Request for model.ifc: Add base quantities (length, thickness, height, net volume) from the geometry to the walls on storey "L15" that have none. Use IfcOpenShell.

First a look at what the model holds.

```python
import ifcopenshell
import ifcopenshell.util.element
import ifcopenshell.util.unit

model = ifcopenshell.open("model.ifc")
print(model.schema)
for unit_type in ("LENGTHUNIT", "AREAUNIT", "VOLUMEUNIT"):
    print(unit_type, ifcopenshell.util.unit.calculate_unit_scale(model, unit_type))
storey = next(s for s in model.by_type("IfcBuildingStorey") if s.Name == "L15")
walls = [e for e in ifcopenshell.util.element.get_decomposition(storey) if e.is_a("IfcWall")]
for e in sorted(walls, key=lambda e: e.id()):
    print(e.id(), e.is_a(), e.Name, list(ifcopenshell.util.element.get_psets(e, qtos_only=True)), sep=" | ")
```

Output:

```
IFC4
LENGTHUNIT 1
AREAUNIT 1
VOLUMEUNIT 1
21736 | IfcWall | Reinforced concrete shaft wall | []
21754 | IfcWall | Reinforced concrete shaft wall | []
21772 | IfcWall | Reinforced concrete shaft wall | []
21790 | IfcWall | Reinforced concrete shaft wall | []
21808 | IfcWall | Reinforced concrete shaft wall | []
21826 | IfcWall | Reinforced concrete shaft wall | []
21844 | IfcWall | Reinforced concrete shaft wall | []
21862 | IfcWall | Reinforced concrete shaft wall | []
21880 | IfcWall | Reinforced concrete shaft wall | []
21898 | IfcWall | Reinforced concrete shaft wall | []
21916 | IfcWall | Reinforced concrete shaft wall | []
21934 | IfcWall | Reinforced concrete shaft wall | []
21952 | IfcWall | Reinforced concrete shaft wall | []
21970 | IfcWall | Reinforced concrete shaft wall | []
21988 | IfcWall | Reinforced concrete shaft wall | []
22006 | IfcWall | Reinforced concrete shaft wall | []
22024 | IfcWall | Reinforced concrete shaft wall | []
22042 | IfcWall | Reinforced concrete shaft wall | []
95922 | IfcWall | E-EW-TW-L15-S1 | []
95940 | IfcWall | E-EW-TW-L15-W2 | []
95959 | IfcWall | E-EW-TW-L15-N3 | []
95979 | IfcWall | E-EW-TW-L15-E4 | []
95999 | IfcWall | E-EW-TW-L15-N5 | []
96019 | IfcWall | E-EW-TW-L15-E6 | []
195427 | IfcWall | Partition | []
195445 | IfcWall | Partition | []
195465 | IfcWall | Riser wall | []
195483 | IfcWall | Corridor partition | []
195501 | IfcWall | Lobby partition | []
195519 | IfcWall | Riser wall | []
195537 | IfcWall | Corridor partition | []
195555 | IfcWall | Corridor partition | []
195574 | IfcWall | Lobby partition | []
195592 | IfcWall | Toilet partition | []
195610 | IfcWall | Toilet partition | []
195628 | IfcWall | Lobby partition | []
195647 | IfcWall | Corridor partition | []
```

```python
import ifcopenshell
import ifcopenshell.api.pset
import ifcopenshell.geom
import ifcopenshell.util.element
import ifcopenshell.util.shape
import ifcopenshell.util.unit

model = ifcopenshell.open("model.ifc")
unit_scale = ifcopenshell.util.unit.calculate_unit_scale(model)
volume_scale = ifcopenshell.util.unit.calculate_unit_scale(model, "VOLUMEUNIT")
settings = ifcopenshell.geom.settings()

storey = next(s for s in model.by_type("IfcBuildingStorey") if s.Name == "L15")
walls = [e for e in ifcopenshell.util.element.get_decomposition(storey) if e.is_a("IfcWall")]

for e in sorted(walls, key=lambda e: e.id()):
    if ifcopenshell.util.element.get_psets(e, qtos_only=True, should_inherit=False):
        continue
    # Geometry comes back in metres, in the element's own axes.
    shape = ifcopenshell.geom.create_shape(settings, e)
    values = {
        "Length": ifcopenshell.util.shape.get_x(shape.geometry) / unit_scale,
        "Width": ifcopenshell.util.shape.get_y(shape.geometry) / unit_scale,
        "Height": ifcopenshell.util.shape.get_z(shape.geometry) / unit_scale,
        "NetVolume": ifcopenshell.util.shape.get_volume(shape.geometry) / volume_scale,
    }
    qto = ifcopenshell.api.pset.add_qto(model, product=e, name="Qto_WallBaseQuantities")
    ifcopenshell.api.pset.edit_qto(model, qto=qto, properties=values)
    print(e.id(), {k: round(v, 3) for k, v in values.items()})

model.write("model_rev.ifc")
```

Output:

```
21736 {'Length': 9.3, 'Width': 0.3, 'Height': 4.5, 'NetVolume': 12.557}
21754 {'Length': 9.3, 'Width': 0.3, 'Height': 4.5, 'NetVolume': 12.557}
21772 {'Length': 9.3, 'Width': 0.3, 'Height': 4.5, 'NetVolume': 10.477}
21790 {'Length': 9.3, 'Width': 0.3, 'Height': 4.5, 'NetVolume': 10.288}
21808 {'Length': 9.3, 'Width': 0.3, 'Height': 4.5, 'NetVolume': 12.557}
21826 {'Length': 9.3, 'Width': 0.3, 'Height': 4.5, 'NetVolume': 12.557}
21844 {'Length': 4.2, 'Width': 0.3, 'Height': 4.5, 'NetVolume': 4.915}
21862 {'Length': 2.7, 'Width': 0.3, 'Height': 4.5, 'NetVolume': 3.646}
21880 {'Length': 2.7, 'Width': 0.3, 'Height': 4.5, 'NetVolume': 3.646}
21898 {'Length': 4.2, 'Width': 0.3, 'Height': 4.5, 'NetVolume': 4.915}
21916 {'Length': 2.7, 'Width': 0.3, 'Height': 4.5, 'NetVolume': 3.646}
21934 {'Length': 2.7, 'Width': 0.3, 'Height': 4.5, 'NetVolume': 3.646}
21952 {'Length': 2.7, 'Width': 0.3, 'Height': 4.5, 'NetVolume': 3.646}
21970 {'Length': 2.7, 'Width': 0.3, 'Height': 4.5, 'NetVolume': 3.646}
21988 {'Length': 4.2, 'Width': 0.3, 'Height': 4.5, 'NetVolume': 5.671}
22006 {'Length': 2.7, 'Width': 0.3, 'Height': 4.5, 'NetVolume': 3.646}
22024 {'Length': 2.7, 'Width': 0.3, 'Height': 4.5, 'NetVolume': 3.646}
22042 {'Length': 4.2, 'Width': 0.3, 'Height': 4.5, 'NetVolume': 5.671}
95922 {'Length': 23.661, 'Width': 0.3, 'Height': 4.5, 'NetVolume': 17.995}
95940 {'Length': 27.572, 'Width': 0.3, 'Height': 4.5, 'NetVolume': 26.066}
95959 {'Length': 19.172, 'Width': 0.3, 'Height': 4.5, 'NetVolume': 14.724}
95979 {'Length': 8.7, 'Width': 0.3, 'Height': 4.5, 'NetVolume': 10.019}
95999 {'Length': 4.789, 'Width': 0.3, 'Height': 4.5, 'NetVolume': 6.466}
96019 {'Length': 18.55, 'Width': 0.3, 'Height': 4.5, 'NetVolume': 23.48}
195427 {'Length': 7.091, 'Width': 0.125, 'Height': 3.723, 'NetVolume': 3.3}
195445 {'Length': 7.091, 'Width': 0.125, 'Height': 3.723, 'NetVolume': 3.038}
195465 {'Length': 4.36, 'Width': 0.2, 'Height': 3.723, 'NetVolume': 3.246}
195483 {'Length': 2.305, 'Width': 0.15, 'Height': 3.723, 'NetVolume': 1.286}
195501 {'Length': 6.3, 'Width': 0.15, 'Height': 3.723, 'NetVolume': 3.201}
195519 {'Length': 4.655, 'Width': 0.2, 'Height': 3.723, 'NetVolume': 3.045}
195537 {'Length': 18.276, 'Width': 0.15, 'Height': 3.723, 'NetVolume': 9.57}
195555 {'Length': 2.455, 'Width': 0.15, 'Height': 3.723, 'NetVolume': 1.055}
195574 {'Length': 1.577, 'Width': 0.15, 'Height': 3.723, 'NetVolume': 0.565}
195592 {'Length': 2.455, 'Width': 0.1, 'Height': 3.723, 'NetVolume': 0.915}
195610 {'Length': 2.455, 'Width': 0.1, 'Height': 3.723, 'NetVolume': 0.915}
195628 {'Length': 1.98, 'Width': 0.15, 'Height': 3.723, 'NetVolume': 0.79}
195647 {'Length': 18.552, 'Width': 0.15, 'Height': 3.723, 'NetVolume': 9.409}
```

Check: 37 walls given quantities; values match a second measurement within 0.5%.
